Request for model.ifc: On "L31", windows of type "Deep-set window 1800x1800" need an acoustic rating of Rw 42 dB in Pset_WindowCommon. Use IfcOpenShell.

First a look at what the model holds.

```python
import ifcopenshell
import ifcopenshell.util.element

model = ifcopenshell.open("model.ifc")
print(model.schema)
storey = next(s for s in model.by_type("IfcBuildingStorey") if s.Name == "L31")
windows = [e for e in ifcopenshell.util.element.get_decomposition(storey) if e.is_a("IfcWindow")]
seen = {}
for e in windows:
    element_type = ifcopenshell.util.element.get_type(e)
    key = (element_type.Name if element_type != e and element_type else None, ifcopenshell.util.element.get_pset(e, "Pset_WindowCommon", "AcousticRating"))
    seen[key] = seen.get(key, 0) + 1
for (name, value), count in sorted(seen.items(), key=str):
    print(count, "x", name, "|", value)
```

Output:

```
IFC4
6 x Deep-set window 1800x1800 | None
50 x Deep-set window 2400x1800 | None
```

```python
import ifcopenshell
import ifcopenshell.api.pset
import ifcopenshell.util.element

model = ifcopenshell.open("model.ifc")

storey = next(s for s in model.by_type("IfcBuildingStorey") if s.Name == "L31")
windows = [e for e in ifcopenshell.util.element.get_decomposition(storey) if e.is_a("IfcWindow")]

count = 0
for e in windows:
    element_type = ifcopenshell.util.element.get_type(e)
    if element_type in (None, e) or element_type.Name != "Deep-set window 1800x1800":
        continue
    found = ifcopenshell.util.element.get_pset(e, "Pset_WindowCommon", should_inherit=False)
    if found:
        pset = model.by_id(found["id"])
        if len(ifcopenshell.util.element.get_elements_by_pset(pset)) > 1:
            pset = ifcopenshell.api.pset.unshare_pset(model, products=[e], pset=pset)[0]
    else:
        pset = ifcopenshell.api.pset.add_pset(model, product=e, name="Pset_WindowCommon")
    ifcopenshell.api.pset.edit_pset(model, pset=pset, properties={"AcousticRating": "Rw 42 dB"})
    count += 1

print(count, "windows updated")

model.write("model-out.ifc")
```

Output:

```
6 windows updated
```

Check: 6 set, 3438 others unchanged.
